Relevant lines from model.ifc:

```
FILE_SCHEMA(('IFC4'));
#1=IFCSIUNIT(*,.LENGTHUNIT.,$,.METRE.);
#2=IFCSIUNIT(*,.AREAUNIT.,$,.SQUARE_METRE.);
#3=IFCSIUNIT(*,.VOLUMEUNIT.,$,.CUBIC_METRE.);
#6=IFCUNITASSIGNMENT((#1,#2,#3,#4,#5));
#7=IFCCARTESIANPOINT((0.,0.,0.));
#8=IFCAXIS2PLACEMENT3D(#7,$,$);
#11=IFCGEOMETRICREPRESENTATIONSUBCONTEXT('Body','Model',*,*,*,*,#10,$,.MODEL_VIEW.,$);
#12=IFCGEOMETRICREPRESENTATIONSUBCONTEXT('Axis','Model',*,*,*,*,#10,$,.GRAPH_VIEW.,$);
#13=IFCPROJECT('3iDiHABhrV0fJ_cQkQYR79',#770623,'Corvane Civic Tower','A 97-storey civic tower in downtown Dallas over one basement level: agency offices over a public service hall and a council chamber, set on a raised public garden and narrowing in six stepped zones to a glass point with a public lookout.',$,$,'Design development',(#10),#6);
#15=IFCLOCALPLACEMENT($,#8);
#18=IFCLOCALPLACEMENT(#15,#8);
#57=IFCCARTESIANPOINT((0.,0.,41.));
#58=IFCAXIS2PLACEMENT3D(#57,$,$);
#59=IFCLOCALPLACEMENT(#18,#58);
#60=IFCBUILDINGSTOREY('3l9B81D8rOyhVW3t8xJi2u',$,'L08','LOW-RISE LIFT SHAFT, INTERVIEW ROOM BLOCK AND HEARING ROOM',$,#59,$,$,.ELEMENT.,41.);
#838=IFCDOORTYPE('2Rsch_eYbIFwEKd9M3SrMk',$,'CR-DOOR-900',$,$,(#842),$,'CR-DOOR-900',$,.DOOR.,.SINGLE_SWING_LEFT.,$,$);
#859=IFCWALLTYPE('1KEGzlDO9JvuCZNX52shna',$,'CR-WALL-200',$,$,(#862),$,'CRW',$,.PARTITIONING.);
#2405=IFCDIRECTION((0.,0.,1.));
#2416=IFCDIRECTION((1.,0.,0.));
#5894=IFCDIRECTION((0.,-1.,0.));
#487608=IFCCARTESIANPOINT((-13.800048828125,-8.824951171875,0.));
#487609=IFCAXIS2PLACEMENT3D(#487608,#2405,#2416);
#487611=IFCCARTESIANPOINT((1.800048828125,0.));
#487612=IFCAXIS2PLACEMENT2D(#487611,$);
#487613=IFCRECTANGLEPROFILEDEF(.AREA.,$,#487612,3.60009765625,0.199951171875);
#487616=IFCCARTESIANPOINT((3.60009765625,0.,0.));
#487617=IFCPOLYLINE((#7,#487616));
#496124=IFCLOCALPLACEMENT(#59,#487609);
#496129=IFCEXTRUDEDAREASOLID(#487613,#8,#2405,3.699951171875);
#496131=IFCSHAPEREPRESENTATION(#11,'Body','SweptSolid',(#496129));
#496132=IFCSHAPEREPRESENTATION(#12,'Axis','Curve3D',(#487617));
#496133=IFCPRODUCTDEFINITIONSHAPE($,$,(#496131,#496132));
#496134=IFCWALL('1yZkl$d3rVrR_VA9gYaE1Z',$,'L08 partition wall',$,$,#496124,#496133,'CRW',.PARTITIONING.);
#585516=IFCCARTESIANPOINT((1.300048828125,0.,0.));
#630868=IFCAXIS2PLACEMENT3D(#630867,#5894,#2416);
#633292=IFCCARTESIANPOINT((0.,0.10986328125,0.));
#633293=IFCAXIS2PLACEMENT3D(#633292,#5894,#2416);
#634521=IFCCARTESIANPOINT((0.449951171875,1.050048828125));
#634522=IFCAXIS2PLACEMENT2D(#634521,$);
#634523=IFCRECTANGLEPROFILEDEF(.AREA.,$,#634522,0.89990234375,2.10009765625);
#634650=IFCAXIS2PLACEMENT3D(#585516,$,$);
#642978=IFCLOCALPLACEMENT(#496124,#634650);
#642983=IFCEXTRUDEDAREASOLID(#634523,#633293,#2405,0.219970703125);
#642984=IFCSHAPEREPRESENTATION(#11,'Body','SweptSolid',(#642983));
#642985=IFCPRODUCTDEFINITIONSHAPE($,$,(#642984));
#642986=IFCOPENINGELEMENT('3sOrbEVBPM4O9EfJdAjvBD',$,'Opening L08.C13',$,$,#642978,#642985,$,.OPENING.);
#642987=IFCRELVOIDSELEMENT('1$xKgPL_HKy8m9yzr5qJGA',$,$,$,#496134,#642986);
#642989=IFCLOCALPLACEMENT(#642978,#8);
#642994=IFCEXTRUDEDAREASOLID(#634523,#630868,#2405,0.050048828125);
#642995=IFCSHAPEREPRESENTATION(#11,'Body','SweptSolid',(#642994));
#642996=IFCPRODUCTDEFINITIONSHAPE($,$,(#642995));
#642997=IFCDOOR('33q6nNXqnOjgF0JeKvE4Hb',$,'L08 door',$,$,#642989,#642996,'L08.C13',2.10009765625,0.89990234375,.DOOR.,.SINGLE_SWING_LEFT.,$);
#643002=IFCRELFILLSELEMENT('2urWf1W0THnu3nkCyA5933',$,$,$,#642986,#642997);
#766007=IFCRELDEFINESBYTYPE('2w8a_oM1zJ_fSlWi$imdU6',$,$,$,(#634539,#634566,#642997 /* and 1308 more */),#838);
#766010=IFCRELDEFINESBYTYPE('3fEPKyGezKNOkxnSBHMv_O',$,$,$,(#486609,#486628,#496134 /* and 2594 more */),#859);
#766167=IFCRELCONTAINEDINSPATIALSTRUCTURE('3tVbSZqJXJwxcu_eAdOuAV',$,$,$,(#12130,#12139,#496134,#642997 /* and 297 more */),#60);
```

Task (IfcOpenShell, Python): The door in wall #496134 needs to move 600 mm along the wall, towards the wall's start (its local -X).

```python
import ifcopenshell
import ifcopenshell.api.geometry
import ifcopenshell.util.placement
import ifcopenshell.util.unit

model = ifcopenshell.open("model.ifc")
unit_scale = ifcopenshell.util.unit.calculate_unit_scale(model)

door = model.by_id(642997)
opening = door.FillsVoids[0].RelatingOpeningElement
wall = opening.VoidsElements[0].RelatingBuildingElement

wall_matrix = ifcopenshell.util.placement.get_local_placement(wall.ObjectPlacement)
shift = wall_matrix[:3, 0] * -0.6 / unit_scale
before = ifcopenshell.util.placement.get_local_placement(door.ObjectPlacement)[:3, 3].copy()

# The door is placed relative to its opening, so it follows when the opening moves.
matrix = ifcopenshell.util.placement.get_local_placement(opening.ObjectPlacement)
matrix[:3, 3] += shift
ifcopenshell.api.geometry.edit_object_placement(
    model, product=opening, matrix=matrix, is_si=False, should_transform_children=True
)

after = ifcopenshell.util.placement.get_local_placement(door.ObjectPlacement)[:3, 3]
print("door moved by", (after - before).round(3) + 0.0)

model.write("model_rev.ifc")
```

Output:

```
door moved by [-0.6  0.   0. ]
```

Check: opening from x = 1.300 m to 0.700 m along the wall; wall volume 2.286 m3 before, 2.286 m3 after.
